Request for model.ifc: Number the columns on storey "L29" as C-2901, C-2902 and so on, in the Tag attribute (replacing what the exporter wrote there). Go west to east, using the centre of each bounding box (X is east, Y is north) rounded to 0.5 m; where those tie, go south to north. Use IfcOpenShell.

First a look at what the model holds.

```python
import ifcopenshell
import ifcopenshell.util.element
import ifcopenshell.util.placement

model = ifcopenshell.open("model.ifc")
print(model.schema)
storey = next(s for s in model.by_type("IfcBuildingStorey") if s.Name == "L29")
columns = [e for e in ifcopenshell.util.element.get_decomposition(storey) if e.is_a("IfcColumn")]
for e in sorted(columns, key=lambda e: e.id()):
    origin = ifcopenshell.util.placement.get_local_placement(e.ObjectPlacement)[:3, 3]
    print(e.id(), e.Tag, e.Name, origin.round(2) + 0.0, sep=" | ")
```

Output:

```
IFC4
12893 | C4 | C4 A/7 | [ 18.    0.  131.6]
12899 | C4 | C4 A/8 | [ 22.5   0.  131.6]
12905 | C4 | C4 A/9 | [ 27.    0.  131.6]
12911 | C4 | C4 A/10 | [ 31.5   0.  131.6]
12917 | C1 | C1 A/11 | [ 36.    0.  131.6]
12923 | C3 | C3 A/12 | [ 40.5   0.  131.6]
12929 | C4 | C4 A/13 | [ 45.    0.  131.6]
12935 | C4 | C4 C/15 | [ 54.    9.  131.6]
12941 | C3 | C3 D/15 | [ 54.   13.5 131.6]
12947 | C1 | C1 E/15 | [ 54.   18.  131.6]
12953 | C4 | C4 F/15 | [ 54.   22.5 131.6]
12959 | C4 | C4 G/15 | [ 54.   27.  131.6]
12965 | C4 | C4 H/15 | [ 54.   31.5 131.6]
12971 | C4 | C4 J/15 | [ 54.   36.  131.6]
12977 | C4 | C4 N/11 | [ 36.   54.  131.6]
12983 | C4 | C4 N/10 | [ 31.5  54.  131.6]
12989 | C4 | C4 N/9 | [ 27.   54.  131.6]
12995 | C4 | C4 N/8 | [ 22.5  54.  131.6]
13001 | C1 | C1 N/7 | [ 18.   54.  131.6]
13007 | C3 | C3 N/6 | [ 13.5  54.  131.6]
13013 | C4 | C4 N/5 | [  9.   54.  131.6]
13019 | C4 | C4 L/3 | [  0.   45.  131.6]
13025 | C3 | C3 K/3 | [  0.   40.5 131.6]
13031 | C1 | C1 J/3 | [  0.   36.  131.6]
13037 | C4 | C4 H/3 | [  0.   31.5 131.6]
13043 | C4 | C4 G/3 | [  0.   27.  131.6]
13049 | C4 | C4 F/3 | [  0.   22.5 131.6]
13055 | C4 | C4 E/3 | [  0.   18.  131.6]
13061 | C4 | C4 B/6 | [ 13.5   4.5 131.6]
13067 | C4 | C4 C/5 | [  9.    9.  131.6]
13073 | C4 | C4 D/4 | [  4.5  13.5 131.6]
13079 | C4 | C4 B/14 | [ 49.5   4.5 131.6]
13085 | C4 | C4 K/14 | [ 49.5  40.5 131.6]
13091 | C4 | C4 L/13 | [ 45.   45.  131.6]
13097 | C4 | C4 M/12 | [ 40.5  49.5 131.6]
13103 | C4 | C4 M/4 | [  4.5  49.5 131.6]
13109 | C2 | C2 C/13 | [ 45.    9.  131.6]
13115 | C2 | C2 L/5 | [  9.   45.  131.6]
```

```python
import ifcopenshell
import ifcopenshell.geom
import ifcopenshell.util.element
import ifcopenshell.util.shape

model = ifcopenshell.open("model.ifc")
settings = ifcopenshell.geom.settings()
settings.set("use-world-coords", True)


def centre(element):
    shape = ifcopenshell.geom.create_shape(settings, element)
    return ifcopenshell.util.shape.get_bbox_centroid(shape.geometry)


storey = next(s for s in model.by_type("IfcBuildingStorey") if s.Name == "L29")
columns = [e for e in ifcopenshell.util.element.get_decomposition(storey) if e.is_a("IfcColumn")]

# Insertion points can sit at a corner or the storey origin, so sort by the geometry (in metres).
centres = {e: centre(e) for e in columns}
columns.sort(key=lambda e: (round(centres[e][0] / 0.5), centres[e][1]))

for i, e in enumerate(columns, start=1):
    number = f"C-29{i:02d}"
    e.Tag = number
    print(e.id(), number)

model.write("model_updated.ifc")
```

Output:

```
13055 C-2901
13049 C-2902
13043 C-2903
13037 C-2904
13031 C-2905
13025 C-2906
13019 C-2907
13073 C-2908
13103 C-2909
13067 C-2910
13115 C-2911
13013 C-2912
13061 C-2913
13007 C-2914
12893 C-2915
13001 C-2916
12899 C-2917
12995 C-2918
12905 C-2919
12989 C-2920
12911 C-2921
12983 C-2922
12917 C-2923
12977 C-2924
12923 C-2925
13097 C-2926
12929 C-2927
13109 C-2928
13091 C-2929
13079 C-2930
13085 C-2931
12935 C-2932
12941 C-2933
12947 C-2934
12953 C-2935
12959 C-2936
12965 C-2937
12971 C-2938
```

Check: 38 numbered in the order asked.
